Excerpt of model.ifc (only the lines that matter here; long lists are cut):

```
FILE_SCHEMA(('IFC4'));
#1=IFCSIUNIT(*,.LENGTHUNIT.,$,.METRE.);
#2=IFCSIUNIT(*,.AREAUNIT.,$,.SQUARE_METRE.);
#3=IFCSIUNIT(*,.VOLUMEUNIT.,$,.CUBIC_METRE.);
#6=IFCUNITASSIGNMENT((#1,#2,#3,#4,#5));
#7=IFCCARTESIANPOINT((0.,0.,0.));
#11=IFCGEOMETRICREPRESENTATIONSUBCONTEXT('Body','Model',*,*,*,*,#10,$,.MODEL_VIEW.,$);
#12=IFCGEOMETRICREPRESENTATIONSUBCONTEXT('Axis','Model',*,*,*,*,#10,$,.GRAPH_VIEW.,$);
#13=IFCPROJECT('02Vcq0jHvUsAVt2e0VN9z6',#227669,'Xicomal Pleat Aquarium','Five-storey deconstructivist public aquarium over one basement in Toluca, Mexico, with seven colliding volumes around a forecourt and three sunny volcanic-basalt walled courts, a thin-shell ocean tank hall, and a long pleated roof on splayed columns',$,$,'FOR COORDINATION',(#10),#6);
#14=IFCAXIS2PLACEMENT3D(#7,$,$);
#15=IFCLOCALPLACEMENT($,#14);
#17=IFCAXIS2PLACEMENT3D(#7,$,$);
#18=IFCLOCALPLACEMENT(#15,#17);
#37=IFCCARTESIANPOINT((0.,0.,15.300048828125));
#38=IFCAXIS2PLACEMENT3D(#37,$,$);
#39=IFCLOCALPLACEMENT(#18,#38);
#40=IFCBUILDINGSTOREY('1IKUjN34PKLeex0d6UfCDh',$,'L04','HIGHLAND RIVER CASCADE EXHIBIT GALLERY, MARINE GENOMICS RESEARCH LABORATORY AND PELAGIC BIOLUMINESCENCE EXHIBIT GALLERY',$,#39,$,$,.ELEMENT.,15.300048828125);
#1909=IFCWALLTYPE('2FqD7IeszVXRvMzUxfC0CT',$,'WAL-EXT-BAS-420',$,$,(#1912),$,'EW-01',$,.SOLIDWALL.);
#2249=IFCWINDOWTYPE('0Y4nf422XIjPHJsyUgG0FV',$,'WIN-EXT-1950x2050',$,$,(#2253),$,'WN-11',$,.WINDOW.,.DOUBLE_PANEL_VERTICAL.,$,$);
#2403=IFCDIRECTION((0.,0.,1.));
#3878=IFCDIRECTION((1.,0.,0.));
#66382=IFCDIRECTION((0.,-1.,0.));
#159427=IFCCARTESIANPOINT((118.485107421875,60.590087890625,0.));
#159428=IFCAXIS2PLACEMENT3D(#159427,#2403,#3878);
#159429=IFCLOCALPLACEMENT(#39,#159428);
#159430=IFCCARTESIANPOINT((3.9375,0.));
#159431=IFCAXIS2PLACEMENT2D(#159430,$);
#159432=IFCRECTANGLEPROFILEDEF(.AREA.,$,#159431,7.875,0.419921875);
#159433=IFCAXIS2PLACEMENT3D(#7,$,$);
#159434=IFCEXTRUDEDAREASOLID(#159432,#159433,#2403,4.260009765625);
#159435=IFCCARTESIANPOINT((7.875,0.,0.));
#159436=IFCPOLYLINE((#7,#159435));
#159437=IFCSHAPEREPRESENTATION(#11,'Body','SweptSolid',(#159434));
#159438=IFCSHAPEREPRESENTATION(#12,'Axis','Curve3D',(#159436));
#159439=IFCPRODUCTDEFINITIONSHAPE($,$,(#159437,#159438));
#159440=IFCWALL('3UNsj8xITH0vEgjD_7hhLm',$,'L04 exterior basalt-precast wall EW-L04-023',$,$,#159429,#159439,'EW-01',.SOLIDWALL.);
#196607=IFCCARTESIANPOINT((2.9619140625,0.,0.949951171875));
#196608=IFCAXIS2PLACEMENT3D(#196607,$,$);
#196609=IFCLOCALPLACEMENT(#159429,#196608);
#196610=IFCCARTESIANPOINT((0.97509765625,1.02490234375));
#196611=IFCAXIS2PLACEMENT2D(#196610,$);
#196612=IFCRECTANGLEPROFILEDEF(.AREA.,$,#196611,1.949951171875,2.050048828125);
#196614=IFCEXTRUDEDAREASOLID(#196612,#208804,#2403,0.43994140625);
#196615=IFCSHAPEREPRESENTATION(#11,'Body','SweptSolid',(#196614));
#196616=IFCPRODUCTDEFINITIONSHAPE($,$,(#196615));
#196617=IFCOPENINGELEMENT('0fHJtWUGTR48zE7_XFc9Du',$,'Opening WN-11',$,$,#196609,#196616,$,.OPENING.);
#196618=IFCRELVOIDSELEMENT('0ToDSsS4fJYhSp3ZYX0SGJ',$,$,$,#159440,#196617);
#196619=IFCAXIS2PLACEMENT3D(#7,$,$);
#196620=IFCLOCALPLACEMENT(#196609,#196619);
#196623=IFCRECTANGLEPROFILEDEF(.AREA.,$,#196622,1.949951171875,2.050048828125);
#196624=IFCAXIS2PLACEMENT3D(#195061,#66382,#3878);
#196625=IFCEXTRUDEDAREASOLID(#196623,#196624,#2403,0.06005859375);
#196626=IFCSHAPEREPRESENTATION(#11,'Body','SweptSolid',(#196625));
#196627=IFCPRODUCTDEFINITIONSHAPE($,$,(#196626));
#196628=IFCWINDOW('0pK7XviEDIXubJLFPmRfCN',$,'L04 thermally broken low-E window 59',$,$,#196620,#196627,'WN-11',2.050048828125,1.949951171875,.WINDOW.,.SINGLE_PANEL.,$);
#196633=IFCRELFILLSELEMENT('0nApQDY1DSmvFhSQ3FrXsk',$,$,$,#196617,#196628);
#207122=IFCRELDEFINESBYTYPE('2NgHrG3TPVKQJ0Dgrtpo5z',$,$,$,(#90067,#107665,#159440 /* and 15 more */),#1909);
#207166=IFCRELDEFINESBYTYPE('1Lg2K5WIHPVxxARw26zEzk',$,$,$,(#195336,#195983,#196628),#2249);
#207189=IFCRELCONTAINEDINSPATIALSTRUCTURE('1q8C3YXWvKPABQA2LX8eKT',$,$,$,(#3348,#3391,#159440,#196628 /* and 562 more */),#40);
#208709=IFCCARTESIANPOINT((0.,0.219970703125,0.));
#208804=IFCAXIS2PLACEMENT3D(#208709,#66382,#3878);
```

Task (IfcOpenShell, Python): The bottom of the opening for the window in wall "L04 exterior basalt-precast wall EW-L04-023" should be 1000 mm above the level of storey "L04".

```python
import numpy as np
import ifcopenshell
import ifcopenshell.api.geometry
import ifcopenshell.geom
import ifcopenshell.util.element
import ifcopenshell.util.placement
import ifcopenshell.util.shape
import ifcopenshell.util.unit

model = ifcopenshell.open("model.ifc")
unit_scale = ifcopenshell.util.unit.calculate_unit_scale(model)

window = model.by_id(196628)
opening = window.FillsVoids[0].RelatingOpeningElement
storey = ifcopenshell.util.element.get_container(window, ifc_class="IfcBuildingStorey")
level = ifcopenshell.util.placement.get_local_placement(storey.ObjectPlacement)[2, 3]

# The opening's origin need not be at the sill, so measure its lowest point.
shape = ifcopenshell.geom.create_shape(ifcopenshell.geom.settings(), opening)
bottom = ifcopenshell.util.shape.get_shape_bottom_elevation(shape, shape.geometry) / unit_scale
dz = level + 1.0 - bottom

shift = np.array([0.0, 0.0, dz])
# The window is placed relative to its opening, so it follows when the opening moves.
matrix = ifcopenshell.util.placement.get_local_placement(opening.ObjectPlacement)
matrix[:3, 3] += shift
ifcopenshell.api.geometry.edit_object_placement(
    model, product=opening, matrix=matrix, is_si=False, should_transform_children=True
)

print(f"moved by {dz * unit_scale:+.3f} m")

model.write("model_rev.ifc")
```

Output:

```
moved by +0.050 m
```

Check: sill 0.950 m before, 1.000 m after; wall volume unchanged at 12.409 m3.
